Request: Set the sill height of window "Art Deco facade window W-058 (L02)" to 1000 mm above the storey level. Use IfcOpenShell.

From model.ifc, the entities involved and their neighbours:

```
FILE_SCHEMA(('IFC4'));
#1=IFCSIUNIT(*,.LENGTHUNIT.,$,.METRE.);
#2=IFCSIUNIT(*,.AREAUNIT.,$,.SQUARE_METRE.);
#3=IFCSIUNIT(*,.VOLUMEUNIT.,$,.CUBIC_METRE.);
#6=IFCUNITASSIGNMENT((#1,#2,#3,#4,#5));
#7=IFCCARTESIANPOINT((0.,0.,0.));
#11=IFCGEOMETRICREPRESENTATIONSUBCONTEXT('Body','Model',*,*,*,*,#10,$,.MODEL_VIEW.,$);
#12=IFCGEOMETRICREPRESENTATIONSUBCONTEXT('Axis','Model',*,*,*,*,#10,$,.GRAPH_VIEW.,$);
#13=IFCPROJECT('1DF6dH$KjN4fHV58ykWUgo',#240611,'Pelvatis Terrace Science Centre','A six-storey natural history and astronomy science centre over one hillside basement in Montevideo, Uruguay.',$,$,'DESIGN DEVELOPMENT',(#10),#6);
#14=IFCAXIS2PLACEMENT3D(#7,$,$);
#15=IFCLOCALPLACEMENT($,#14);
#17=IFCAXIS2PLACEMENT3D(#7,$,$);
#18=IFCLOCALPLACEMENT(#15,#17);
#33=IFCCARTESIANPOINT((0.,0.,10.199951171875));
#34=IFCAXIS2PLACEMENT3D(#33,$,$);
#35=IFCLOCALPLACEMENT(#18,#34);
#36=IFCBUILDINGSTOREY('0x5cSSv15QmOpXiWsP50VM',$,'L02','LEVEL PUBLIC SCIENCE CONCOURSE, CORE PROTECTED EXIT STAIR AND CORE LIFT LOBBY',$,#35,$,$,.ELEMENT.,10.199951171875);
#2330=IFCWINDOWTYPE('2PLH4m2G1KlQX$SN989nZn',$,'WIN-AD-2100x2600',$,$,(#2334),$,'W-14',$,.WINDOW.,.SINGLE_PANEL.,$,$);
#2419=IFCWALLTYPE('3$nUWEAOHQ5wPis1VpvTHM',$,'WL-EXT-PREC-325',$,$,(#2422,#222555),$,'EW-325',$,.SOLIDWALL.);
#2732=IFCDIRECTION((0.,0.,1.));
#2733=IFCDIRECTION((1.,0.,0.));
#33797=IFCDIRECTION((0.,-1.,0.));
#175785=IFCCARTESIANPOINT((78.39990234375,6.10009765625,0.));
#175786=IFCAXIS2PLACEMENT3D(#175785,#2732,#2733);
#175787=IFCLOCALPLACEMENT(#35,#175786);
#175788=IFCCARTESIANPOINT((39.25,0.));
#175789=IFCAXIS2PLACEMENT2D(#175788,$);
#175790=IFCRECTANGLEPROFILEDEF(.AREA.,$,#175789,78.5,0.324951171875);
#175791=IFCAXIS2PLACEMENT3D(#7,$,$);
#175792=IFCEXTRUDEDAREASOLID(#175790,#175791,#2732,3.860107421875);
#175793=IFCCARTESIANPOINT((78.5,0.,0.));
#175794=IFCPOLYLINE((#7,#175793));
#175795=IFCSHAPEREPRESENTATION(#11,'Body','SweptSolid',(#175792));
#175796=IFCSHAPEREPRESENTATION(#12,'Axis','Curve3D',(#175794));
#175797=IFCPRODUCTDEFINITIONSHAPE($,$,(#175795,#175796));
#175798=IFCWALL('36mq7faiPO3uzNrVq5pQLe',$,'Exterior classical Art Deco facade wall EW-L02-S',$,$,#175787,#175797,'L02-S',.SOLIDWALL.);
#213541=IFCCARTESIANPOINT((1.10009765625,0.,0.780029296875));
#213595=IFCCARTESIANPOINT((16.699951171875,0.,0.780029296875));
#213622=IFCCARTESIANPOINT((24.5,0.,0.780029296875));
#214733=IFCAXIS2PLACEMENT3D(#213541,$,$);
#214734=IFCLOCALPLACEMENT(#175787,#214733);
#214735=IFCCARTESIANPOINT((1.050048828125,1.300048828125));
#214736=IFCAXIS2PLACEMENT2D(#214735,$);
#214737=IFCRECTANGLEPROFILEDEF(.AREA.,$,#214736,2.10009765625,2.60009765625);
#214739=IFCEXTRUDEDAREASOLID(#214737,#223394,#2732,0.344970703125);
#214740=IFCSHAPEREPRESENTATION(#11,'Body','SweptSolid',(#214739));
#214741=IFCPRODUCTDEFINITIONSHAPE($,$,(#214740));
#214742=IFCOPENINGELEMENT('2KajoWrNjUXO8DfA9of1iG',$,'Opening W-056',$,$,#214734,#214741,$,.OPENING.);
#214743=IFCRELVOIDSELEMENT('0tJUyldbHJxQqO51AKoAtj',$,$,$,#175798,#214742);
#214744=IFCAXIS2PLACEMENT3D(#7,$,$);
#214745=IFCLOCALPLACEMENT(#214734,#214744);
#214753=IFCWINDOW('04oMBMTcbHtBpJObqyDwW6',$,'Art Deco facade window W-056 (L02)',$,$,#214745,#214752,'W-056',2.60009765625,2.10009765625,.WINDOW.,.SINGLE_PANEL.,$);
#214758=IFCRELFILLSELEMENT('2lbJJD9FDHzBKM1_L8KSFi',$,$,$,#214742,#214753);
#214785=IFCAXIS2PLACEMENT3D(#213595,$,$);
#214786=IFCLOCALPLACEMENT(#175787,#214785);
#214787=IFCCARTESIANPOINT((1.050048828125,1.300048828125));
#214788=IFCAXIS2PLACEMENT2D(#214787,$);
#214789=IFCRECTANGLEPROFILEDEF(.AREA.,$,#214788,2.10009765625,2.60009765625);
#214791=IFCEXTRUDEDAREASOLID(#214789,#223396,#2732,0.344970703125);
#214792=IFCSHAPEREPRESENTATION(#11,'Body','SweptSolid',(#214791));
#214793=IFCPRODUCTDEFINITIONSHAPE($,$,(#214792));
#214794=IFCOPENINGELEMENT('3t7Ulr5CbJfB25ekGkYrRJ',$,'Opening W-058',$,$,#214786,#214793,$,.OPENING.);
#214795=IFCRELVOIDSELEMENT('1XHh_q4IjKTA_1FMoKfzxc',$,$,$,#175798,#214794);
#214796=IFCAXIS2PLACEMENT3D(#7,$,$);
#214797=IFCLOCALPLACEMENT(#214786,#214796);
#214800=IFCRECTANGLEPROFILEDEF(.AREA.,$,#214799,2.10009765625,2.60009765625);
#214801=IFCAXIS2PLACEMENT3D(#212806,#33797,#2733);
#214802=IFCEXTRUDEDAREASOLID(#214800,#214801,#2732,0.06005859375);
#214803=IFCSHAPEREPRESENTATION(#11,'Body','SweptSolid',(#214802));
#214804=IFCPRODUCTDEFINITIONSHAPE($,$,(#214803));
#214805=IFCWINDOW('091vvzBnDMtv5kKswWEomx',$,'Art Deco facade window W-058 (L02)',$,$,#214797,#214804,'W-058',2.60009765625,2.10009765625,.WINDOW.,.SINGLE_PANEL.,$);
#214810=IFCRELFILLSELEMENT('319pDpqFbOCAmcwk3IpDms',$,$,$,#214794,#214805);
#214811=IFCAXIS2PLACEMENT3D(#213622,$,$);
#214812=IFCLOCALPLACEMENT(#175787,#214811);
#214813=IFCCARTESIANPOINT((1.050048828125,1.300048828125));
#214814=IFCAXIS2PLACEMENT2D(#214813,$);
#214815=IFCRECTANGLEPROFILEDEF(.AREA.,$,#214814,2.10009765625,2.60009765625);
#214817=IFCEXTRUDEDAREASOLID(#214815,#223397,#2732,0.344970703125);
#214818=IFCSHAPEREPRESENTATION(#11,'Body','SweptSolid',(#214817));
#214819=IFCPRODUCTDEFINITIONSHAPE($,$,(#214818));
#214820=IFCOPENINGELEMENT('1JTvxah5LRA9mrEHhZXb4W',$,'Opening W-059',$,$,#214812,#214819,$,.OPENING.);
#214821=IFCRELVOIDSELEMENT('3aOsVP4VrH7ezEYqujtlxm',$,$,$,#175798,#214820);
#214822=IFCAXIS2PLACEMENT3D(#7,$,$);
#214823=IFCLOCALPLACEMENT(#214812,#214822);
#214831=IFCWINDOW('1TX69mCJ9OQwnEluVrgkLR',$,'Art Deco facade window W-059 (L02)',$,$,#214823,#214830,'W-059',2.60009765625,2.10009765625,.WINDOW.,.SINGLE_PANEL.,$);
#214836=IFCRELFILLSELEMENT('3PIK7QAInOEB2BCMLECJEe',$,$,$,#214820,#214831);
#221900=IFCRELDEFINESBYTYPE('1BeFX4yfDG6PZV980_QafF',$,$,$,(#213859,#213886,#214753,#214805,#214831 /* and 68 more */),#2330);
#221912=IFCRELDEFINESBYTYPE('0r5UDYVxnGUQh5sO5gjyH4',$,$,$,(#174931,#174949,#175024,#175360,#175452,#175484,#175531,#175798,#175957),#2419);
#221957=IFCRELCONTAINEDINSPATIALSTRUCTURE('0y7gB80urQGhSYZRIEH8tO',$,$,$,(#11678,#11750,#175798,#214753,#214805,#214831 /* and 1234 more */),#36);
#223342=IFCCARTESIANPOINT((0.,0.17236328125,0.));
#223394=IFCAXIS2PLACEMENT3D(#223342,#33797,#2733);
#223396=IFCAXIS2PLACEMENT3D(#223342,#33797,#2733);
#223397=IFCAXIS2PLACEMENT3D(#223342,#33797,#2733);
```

```python
import numpy as np
import ifcopenshell
import ifcopenshell.api.geometry
import ifcopenshell.geom
import ifcopenshell.util.element
import ifcopenshell.util.placement
import ifcopenshell.util.shape
import ifcopenshell.util.unit

model = ifcopenshell.open("model.ifc")
unit_scale = ifcopenshell.util.unit.calculate_unit_scale(model)

window = model.by_guid("091vvzBnDMtv5kKswWEomx")
opening = window.FillsVoids[0].RelatingOpeningElement
storey = ifcopenshell.util.element.get_container(window, ifc_class="IfcBuildingStorey")
level = ifcopenshell.util.placement.get_local_placement(storey.ObjectPlacement)[2, 3]

# The opening's origin need not be at the sill, so measure its lowest point.
shape = ifcopenshell.geom.create_shape(ifcopenshell.geom.settings(), opening)
bottom = ifcopenshell.util.shape.get_shape_bottom_elevation(shape, shape.geometry) / unit_scale
dz = level + 1 / unit_scale - bottom

shift = np.array([0.0, 0.0, dz])
# The window is placed relative to its opening, so it follows when the opening moves.
matrix = ifcopenshell.util.placement.get_local_placement(opening.ObjectPlacement)
matrix[:3, 3] += shift
ifcopenshell.api.geometry.edit_object_placement(
    model, product=opening, matrix=matrix, is_si=False, should_transform_children=True
)

print(f"moved by {dz * unit_scale:+.3f} m")

model.write("model-out.ifc")
```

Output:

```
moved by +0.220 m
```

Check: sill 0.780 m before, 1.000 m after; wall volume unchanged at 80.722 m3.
